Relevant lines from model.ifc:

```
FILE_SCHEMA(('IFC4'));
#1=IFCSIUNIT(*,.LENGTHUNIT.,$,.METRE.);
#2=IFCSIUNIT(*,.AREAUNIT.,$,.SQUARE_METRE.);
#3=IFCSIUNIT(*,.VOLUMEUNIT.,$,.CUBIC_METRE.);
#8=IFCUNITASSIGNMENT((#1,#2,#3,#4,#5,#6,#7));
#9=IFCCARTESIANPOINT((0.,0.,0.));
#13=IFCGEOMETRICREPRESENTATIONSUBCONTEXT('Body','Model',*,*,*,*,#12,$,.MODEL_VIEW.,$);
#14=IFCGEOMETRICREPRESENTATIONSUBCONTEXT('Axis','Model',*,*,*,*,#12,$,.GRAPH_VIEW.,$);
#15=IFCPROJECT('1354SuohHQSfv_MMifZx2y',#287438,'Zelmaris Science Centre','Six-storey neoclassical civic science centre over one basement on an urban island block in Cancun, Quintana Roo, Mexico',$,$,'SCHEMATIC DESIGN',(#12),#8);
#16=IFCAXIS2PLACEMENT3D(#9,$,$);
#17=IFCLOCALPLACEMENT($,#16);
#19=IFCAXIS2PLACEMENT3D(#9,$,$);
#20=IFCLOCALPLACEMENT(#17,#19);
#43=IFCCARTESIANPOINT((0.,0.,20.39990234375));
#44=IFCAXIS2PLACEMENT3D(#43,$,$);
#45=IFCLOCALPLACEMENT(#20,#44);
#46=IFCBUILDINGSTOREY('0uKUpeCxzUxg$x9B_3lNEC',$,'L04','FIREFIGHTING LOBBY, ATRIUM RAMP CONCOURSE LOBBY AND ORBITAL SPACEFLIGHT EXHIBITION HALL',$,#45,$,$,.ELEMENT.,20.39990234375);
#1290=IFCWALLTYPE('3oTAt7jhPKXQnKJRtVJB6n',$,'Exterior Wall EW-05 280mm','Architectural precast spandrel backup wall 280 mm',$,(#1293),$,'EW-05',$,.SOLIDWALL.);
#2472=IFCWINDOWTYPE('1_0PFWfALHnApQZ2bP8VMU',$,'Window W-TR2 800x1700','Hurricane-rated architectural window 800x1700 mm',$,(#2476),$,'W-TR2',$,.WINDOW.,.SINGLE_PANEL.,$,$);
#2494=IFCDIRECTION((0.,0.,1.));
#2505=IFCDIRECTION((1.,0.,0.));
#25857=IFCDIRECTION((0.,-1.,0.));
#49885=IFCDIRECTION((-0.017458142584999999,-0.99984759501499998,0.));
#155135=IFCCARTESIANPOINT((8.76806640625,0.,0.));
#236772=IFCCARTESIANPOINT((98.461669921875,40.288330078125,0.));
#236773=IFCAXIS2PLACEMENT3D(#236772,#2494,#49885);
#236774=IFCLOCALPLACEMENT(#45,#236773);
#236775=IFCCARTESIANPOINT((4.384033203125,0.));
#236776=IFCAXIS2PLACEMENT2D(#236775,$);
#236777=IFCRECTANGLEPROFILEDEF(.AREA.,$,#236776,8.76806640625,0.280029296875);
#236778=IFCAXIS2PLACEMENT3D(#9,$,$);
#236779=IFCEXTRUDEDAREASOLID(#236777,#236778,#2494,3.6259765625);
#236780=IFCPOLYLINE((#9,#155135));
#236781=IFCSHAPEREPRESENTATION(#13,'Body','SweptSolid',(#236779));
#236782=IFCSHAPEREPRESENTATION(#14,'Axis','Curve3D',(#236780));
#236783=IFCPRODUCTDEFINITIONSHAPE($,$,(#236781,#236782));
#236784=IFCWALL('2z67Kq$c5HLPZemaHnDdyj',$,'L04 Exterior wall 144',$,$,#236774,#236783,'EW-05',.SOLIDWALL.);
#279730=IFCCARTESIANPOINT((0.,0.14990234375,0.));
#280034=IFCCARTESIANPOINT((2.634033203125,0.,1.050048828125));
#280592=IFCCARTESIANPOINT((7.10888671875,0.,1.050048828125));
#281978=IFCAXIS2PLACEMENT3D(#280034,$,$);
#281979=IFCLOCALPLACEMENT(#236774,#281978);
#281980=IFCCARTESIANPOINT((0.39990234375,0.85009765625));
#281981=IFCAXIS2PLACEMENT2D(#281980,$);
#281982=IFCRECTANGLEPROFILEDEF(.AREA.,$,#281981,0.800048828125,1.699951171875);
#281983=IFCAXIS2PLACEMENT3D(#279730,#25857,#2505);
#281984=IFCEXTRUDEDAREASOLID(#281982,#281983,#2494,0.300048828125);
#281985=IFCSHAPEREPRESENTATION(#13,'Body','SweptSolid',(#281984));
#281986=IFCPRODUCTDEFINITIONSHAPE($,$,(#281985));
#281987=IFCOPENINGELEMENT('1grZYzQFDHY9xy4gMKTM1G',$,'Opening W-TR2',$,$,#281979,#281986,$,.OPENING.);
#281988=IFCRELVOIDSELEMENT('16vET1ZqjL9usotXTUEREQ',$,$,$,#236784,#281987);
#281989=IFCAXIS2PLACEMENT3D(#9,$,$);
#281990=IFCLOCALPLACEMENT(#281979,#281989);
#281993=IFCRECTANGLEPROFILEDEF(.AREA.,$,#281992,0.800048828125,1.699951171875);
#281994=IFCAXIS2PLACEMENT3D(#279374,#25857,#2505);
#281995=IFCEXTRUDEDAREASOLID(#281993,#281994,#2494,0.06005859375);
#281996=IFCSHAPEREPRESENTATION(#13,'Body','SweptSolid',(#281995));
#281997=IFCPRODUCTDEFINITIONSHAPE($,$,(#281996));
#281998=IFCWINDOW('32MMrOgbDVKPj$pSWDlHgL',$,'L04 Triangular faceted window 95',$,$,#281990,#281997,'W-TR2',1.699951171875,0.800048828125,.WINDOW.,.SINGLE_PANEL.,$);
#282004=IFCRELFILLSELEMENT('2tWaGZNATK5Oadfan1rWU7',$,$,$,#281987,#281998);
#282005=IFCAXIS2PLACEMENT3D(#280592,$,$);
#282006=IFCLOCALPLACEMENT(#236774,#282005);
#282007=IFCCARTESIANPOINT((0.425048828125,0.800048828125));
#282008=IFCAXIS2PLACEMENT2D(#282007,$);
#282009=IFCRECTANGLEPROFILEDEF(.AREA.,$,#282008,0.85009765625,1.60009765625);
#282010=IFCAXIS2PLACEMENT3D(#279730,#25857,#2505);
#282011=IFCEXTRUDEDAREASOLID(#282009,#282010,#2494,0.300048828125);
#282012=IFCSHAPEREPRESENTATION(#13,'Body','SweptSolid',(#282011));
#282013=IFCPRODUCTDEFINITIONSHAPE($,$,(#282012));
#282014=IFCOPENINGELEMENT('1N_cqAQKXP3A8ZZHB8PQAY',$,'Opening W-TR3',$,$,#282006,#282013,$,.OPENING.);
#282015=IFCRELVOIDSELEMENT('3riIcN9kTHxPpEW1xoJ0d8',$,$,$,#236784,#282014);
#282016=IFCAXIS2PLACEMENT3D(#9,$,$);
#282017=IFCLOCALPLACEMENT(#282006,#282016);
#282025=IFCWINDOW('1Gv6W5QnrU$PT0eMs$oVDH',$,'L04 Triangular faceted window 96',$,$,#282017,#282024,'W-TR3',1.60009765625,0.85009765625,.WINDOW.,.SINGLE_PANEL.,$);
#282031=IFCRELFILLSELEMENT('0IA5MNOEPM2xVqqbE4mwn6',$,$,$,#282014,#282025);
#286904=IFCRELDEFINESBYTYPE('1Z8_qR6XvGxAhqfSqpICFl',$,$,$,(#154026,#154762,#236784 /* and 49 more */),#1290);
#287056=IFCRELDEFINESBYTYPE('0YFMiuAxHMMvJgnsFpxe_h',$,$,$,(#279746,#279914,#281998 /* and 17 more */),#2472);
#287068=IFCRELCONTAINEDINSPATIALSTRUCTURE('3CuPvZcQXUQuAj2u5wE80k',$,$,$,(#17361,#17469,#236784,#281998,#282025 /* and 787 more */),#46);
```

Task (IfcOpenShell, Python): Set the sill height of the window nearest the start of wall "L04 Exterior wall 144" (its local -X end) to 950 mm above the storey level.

```python
import numpy as np
import ifcopenshell
import ifcopenshell.api.geometry
import ifcopenshell.geom
import ifcopenshell.util.element
import ifcopenshell.util.placement
import ifcopenshell.util.shape
import ifcopenshell.util.unit

model = ifcopenshell.open("model.ifc")
unit_scale = ifcopenshell.util.unit.calculate_unit_scale(model)

window = model.by_guid("32MMrOgbDVKPj$pSWDlHgL")
opening = window.FillsVoids[0].RelatingOpeningElement
storey = ifcopenshell.util.element.get_container(window, ifc_class="IfcBuildingStorey")
level = ifcopenshell.util.placement.get_local_placement(storey.ObjectPlacement)[2, 3]

# The opening's origin need not be at the sill, so measure its lowest point.
shape = ifcopenshell.geom.create_shape(ifcopenshell.geom.settings(), opening)
bottom = ifcopenshell.util.shape.get_shape_bottom_elevation(shape, shape.geometry) / unit_scale
dz = level + 0.95 / unit_scale - bottom

shift = np.array([0.0, 0.0, dz])
# The window is placed relative to its opening, so it follows when the opening moves.
matrix = ifcopenshell.util.placement.get_local_placement(opening.ObjectPlacement)
matrix[:3, 3] += shift
ifcopenshell.api.geometry.edit_object_placement(
    model, product=opening, matrix=matrix, is_si=False, should_transform_children=True
)

print(f"moved by {dz * unit_scale:+.3f} m")

model.write("model_rev.ifc")
```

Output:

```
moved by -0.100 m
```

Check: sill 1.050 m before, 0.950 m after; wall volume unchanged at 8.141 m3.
